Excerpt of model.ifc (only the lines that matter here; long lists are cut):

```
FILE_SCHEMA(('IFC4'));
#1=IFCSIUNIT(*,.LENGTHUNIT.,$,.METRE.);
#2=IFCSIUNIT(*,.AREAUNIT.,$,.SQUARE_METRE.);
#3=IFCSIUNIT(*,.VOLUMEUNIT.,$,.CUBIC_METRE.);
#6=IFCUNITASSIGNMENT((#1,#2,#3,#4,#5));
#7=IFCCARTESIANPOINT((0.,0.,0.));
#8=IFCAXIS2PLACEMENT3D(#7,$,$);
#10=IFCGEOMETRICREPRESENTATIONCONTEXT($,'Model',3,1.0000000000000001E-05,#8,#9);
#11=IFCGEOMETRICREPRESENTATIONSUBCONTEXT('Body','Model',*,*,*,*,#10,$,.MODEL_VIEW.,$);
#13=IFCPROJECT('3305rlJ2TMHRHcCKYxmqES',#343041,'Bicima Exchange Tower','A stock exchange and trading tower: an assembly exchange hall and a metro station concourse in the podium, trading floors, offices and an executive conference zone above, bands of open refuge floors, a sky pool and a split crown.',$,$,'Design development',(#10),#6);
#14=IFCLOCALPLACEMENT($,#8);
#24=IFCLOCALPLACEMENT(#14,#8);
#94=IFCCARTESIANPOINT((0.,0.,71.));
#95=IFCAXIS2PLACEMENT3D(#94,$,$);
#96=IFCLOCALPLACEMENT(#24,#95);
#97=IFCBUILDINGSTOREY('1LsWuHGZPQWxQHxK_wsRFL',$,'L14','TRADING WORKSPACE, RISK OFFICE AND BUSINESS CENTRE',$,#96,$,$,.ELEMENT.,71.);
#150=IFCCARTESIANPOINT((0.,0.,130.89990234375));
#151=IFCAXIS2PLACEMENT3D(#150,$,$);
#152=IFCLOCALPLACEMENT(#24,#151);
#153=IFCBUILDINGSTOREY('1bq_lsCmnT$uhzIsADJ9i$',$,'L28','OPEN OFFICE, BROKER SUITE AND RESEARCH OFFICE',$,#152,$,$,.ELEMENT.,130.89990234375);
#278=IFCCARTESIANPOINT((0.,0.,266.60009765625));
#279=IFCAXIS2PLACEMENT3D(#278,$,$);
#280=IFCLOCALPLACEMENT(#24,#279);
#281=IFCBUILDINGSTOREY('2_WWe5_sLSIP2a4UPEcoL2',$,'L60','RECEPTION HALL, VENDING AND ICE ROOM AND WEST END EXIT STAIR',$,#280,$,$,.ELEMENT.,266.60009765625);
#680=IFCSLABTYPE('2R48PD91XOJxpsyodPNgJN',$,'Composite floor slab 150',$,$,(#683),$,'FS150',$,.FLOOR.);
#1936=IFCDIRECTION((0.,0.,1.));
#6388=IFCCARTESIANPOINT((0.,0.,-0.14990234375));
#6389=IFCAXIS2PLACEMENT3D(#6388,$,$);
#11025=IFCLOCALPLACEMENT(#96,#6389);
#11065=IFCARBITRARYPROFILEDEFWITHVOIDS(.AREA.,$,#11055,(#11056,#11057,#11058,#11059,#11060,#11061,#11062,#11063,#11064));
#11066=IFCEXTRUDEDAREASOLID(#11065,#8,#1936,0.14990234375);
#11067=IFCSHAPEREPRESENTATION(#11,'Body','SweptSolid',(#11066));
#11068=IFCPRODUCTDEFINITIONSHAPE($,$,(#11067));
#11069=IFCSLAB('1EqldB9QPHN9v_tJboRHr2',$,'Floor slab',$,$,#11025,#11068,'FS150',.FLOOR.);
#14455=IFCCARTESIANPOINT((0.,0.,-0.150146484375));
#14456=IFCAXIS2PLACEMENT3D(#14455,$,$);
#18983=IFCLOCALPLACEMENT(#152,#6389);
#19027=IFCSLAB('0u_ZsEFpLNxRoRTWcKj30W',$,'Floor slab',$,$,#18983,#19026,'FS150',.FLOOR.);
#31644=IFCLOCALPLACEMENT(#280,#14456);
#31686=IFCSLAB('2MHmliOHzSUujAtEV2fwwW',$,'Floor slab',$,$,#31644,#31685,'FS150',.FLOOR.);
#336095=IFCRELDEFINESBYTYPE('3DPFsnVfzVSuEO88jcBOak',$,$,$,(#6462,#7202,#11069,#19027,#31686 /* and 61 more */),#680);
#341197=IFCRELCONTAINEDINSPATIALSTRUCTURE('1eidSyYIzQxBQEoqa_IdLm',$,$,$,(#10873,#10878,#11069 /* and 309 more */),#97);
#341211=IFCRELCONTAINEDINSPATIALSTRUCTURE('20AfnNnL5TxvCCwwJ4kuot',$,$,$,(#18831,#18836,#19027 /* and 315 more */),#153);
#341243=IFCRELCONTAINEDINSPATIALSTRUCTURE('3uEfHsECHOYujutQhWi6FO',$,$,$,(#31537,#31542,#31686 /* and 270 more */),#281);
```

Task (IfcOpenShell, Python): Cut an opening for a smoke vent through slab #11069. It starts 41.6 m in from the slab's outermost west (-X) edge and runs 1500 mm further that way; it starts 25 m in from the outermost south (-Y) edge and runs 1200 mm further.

```python
import numpy as np
import ifcopenshell
import ifcopenshell.api.feature
import ifcopenshell.api.geometry
import ifcopenshell.api.root
import ifcopenshell.geom
import ifcopenshell.util.placement
import ifcopenshell.util.representation
import ifcopenshell.util.shape
import ifcopenshell.util.unit

model = ifcopenshell.open("model.ifc")
unit_scale = ifcopenshell.util.unit.calculate_unit_scale(model)
settings = ifcopenshell.geom.settings()


def volume(element):
    """Net volume in cubic metres, openings subtracted."""
    shape = ifcopenshell.geom.create_shape(settings, element)
    return ifcopenshell.util.shape.get_volume(shape.geometry)


slab = model.by_id(11069)
before = volume(slab)

# Extent in the slab's own axes, in metres. The edges named are its -X and -Y sides.
slab_shape = ifcopenshell.geom.create_shape(settings, slab)
vertices = ifcopenshell.util.shape.get_vertices(slab_shape.geometry)
x_min, y_min, bottom = vertices.min(axis=0)
top = vertices[:, 2].max()

opening = ifcopenshell.api.root.create_entity(model, ifc_class="IfcOpeningElement", name="Smoke vent opening", predefined_type="OPENING")
context = ifcopenshell.util.representation.get_context(model, "Model", "Body", "MODEL_VIEW")
width, depth = 1.5, 1.2
outline = [(0.0, 0.0), (width, 0.0), (width, depth), (0.0, depth), (0.0, 0.0)]
# Overshoot both faces by 50 mm so the cut is clean.
shape = ifcopenshell.api.geometry.add_slab_representation(
    model, context=context, depth=top - bottom + 0.1, polyline=outline
)
ifcopenshell.api.geometry.assign_representation(model, product=opening, representation=shape)

matrix = ifcopenshell.util.placement.get_local_placement(slab.ObjectPlacement)
matrix[:, 3] = matrix @ np.append(np.array([x_min + 41.6, y_min + 25, bottom - 0.05]) / unit_scale, 1.0)
ifcopenshell.api.geometry.edit_object_placement(model, product=opening, matrix=matrix, is_si=False)
ifcopenshell.api.feature.add_feature(model, feature=opening, element=slab)

after = volume(slab)

print(f"slab volume {before:.3f} -> {after:.3f} m3")

model.write("model-out.ifc")
```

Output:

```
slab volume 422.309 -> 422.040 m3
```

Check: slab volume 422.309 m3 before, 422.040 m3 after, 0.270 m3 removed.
